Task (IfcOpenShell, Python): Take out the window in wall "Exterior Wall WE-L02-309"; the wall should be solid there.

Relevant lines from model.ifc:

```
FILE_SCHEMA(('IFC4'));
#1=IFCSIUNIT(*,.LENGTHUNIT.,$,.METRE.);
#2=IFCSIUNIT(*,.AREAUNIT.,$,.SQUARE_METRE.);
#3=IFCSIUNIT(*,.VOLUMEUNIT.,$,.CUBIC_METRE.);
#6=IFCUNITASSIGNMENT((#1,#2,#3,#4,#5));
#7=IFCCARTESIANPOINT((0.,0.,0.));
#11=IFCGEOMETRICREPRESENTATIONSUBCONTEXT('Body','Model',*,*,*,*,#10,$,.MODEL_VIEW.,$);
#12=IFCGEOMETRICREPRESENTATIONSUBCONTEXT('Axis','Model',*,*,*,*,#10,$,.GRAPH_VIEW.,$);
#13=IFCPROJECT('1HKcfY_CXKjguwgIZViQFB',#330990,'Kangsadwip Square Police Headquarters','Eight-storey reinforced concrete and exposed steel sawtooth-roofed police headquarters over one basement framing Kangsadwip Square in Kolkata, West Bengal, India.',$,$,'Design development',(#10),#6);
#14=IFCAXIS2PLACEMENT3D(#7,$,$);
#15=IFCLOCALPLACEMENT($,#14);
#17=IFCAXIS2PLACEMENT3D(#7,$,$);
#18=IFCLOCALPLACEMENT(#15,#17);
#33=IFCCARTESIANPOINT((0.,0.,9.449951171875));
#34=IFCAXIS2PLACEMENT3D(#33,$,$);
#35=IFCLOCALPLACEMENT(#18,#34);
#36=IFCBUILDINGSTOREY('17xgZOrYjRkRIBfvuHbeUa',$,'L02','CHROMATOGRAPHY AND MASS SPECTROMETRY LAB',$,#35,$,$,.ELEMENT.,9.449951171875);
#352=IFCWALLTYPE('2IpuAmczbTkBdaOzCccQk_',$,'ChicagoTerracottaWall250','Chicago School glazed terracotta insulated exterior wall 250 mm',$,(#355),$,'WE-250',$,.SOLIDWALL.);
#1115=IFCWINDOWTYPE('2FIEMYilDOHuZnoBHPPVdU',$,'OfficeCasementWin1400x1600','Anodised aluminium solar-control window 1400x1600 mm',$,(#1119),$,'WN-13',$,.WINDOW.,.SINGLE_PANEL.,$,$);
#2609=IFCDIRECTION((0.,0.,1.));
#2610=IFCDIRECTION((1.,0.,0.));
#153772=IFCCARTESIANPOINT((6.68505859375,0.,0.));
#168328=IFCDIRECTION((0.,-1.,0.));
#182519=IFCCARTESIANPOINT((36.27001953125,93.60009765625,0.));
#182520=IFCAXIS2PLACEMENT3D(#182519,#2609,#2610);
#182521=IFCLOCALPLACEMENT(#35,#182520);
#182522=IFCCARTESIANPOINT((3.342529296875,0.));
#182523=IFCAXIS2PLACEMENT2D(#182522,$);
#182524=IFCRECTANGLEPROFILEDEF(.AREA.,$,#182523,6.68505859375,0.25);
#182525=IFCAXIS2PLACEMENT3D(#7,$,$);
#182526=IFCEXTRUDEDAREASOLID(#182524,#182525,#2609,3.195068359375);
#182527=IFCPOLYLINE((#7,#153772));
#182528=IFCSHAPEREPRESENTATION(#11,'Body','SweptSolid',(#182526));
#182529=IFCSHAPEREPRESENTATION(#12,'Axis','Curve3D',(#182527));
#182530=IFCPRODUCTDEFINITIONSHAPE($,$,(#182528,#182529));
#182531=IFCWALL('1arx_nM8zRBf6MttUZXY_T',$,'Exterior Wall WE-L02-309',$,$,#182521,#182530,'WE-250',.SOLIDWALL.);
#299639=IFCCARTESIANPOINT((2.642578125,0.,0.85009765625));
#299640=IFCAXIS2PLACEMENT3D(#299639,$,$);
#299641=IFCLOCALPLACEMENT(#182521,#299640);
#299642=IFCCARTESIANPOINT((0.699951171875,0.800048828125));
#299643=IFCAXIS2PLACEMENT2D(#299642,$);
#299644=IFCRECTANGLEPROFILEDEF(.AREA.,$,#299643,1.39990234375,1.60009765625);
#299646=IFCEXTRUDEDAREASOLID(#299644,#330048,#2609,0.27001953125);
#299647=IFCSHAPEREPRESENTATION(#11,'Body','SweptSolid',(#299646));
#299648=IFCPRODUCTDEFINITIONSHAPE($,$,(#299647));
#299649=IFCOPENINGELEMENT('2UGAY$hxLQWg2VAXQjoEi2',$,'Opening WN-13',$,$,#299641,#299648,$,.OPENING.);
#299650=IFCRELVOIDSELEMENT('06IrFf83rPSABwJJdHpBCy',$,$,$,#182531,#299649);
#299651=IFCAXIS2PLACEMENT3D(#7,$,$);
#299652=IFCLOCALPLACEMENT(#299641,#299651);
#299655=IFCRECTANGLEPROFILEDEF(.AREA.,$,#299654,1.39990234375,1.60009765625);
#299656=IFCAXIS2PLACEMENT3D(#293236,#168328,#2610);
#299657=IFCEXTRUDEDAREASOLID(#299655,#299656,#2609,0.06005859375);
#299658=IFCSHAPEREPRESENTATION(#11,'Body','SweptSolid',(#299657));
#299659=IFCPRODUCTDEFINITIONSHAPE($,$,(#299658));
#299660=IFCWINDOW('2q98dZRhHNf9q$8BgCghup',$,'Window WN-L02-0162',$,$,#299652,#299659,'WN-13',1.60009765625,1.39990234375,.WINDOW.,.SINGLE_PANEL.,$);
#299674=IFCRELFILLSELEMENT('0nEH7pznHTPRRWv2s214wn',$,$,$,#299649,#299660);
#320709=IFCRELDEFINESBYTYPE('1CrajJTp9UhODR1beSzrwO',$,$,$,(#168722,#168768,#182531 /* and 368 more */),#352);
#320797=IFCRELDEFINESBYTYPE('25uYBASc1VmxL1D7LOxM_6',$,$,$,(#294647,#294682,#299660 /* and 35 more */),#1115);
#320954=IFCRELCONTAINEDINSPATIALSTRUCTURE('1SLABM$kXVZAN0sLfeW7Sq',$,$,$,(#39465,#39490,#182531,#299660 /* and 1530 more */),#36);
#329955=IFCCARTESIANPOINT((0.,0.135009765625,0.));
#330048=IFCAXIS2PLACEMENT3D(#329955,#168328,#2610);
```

```python
import ifcopenshell
import ifcopenshell.api.feature
import ifcopenshell.api.root
import ifcopenshell.geom
import ifcopenshell.util.shape

model = ifcopenshell.open("model.ifc")
settings = ifcopenshell.geom.settings()


def volume(element):
    """Net volume in cubic metres, openings subtracted."""
    shape = ifcopenshell.geom.create_shape(settings, element)
    return ifcopenshell.util.shape.get_volume(shape.geometry)


window = model.by_guid("2q98dZRhHNf9q$8BgCghup")
opening = window.FillsVoids[0].RelatingOpeningElement
wall = opening.VoidsElements[0].RelatingBuildingElement
before = volume(wall)

ifcopenshell.api.root.remove_product(model, product=window)
ifcopenshell.api.feature.remove_feature(model, feature=opening)

after = volume(wall)

print(f"wall volume {before:.3f} -> {after:.3f} m3")

model.write("model_rev.ifc")
```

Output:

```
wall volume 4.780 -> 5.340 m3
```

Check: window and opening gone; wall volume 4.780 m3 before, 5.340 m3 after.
